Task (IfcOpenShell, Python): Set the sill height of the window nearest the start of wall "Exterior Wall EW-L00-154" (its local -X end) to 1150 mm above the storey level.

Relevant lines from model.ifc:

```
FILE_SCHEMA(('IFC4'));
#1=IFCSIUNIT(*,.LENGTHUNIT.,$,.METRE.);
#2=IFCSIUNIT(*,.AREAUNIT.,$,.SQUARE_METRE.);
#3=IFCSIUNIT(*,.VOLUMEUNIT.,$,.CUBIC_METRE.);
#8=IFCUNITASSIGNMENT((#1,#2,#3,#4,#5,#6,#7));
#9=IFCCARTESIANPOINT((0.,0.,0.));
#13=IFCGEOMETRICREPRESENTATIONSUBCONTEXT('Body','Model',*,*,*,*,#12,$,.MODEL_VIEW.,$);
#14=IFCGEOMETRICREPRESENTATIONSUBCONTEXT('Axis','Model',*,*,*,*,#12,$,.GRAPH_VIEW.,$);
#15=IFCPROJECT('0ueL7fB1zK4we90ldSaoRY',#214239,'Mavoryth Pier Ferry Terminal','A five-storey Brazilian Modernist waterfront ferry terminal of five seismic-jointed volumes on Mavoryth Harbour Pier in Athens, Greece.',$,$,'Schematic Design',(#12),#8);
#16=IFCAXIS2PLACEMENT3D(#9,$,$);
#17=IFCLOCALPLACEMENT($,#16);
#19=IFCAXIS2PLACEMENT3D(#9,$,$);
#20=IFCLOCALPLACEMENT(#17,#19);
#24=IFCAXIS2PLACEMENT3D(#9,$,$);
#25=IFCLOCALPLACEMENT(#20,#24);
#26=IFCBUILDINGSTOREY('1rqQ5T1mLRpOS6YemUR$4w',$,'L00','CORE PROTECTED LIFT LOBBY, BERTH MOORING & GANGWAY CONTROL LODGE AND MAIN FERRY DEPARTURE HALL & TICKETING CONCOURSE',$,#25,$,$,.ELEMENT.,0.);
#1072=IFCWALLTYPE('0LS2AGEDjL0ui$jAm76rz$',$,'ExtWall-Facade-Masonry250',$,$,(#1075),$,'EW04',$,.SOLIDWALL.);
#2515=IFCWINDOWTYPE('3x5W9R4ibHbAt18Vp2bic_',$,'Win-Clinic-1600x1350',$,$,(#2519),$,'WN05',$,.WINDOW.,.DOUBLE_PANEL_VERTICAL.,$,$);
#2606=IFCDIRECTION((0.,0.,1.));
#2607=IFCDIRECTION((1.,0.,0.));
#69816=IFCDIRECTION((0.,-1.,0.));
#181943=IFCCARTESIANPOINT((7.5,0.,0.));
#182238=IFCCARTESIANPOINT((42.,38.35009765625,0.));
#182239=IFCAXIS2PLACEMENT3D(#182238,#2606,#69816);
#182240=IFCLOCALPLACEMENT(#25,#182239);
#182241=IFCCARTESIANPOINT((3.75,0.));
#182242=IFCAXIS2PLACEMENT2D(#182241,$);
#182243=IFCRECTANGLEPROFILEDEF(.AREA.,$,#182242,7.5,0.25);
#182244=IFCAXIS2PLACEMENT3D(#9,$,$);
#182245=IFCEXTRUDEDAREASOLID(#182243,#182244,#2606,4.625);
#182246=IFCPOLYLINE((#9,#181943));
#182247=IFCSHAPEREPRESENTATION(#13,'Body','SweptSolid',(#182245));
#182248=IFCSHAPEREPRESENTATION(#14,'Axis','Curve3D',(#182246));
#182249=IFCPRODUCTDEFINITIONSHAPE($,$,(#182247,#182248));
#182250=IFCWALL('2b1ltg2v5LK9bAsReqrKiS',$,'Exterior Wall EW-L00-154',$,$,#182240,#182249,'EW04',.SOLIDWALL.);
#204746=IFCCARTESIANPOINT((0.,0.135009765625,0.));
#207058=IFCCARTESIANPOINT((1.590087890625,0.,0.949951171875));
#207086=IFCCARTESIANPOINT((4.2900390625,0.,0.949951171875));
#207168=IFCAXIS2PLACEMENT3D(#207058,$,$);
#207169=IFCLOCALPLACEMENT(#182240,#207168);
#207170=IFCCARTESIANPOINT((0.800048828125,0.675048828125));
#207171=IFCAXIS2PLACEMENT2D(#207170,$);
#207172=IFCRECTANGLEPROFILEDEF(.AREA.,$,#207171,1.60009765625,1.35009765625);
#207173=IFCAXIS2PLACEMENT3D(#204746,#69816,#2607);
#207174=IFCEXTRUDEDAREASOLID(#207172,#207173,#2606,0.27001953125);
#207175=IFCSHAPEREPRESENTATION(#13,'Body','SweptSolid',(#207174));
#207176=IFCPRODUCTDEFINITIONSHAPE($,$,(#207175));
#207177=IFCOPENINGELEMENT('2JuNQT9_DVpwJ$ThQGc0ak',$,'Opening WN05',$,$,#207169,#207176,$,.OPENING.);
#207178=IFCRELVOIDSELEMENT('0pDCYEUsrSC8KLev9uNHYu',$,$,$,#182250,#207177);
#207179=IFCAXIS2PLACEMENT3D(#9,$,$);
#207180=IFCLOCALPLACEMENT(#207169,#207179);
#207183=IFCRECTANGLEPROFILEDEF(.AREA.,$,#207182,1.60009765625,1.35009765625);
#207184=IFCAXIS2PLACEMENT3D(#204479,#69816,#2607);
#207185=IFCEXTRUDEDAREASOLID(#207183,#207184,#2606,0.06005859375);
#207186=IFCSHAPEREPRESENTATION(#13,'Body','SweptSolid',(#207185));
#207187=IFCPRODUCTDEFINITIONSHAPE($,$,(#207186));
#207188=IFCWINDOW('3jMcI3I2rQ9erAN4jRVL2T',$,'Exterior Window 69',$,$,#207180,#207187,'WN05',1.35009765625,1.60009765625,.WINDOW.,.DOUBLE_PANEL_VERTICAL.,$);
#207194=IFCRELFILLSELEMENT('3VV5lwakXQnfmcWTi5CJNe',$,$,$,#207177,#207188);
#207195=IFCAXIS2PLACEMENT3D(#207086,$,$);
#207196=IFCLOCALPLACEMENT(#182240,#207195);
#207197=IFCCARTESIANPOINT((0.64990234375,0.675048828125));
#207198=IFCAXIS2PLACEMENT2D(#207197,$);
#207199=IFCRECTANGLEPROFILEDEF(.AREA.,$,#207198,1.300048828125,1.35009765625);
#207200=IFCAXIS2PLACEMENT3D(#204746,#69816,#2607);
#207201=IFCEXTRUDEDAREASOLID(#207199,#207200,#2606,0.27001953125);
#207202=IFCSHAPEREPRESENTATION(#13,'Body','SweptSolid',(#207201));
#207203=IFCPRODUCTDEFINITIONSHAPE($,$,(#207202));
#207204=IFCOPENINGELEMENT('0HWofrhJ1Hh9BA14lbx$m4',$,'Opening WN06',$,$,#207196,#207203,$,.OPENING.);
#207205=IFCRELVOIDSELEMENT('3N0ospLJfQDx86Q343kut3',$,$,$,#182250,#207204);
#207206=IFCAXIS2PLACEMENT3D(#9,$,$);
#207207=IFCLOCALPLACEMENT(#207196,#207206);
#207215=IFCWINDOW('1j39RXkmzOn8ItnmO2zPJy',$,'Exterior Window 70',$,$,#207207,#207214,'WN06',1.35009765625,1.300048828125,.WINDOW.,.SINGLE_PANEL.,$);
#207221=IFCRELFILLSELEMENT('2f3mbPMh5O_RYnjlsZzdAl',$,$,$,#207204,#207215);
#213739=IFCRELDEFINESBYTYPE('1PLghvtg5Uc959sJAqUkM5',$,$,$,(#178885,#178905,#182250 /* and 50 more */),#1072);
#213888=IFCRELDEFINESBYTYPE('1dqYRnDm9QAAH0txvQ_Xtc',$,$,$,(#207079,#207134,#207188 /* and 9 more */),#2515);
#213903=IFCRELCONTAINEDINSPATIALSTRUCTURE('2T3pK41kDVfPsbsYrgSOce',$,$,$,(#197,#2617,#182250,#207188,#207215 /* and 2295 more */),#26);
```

```python
import numpy as np
import ifcopenshell
import ifcopenshell.api.geometry
import ifcopenshell.geom
import ifcopenshell.util.element
import ifcopenshell.util.placement
import ifcopenshell.util.shape
import ifcopenshell.util.unit

model = ifcopenshell.open("model.ifc")
unit_scale = ifcopenshell.util.unit.calculate_unit_scale(model)

window = model.by_guid("3jMcI3I2rQ9erAN4jRVL2T")
opening = window.FillsVoids[0].RelatingOpeningElement
storey = ifcopenshell.util.element.get_container(window, ifc_class="IfcBuildingStorey")
level = ifcopenshell.util.placement.get_local_placement(storey.ObjectPlacement)[2, 3]

# The opening's origin need not be at the sill, so measure its lowest point.
shape = ifcopenshell.geom.create_shape(ifcopenshell.geom.settings(), opening)
bottom = ifcopenshell.util.shape.get_shape_bottom_elevation(shape, shape.geometry) / unit_scale
dz = level + 1.15 / unit_scale - bottom

shift = np.array([0.0, 0.0, dz])
# The window is placed relative to its opening, so it follows when the opening moves.
matrix = ifcopenshell.util.placement.get_local_placement(opening.ObjectPlacement)
matrix[:3, 3] += shift
ifcopenshell.api.geometry.edit_object_placement(
    model, product=opening, matrix=matrix, is_si=False, should_transform_children=True
)

print(f"moved by {dz * unit_scale:+.3f} m")

model.write("model_updated.ifc")
```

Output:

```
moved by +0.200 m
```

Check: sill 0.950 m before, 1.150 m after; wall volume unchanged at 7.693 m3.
